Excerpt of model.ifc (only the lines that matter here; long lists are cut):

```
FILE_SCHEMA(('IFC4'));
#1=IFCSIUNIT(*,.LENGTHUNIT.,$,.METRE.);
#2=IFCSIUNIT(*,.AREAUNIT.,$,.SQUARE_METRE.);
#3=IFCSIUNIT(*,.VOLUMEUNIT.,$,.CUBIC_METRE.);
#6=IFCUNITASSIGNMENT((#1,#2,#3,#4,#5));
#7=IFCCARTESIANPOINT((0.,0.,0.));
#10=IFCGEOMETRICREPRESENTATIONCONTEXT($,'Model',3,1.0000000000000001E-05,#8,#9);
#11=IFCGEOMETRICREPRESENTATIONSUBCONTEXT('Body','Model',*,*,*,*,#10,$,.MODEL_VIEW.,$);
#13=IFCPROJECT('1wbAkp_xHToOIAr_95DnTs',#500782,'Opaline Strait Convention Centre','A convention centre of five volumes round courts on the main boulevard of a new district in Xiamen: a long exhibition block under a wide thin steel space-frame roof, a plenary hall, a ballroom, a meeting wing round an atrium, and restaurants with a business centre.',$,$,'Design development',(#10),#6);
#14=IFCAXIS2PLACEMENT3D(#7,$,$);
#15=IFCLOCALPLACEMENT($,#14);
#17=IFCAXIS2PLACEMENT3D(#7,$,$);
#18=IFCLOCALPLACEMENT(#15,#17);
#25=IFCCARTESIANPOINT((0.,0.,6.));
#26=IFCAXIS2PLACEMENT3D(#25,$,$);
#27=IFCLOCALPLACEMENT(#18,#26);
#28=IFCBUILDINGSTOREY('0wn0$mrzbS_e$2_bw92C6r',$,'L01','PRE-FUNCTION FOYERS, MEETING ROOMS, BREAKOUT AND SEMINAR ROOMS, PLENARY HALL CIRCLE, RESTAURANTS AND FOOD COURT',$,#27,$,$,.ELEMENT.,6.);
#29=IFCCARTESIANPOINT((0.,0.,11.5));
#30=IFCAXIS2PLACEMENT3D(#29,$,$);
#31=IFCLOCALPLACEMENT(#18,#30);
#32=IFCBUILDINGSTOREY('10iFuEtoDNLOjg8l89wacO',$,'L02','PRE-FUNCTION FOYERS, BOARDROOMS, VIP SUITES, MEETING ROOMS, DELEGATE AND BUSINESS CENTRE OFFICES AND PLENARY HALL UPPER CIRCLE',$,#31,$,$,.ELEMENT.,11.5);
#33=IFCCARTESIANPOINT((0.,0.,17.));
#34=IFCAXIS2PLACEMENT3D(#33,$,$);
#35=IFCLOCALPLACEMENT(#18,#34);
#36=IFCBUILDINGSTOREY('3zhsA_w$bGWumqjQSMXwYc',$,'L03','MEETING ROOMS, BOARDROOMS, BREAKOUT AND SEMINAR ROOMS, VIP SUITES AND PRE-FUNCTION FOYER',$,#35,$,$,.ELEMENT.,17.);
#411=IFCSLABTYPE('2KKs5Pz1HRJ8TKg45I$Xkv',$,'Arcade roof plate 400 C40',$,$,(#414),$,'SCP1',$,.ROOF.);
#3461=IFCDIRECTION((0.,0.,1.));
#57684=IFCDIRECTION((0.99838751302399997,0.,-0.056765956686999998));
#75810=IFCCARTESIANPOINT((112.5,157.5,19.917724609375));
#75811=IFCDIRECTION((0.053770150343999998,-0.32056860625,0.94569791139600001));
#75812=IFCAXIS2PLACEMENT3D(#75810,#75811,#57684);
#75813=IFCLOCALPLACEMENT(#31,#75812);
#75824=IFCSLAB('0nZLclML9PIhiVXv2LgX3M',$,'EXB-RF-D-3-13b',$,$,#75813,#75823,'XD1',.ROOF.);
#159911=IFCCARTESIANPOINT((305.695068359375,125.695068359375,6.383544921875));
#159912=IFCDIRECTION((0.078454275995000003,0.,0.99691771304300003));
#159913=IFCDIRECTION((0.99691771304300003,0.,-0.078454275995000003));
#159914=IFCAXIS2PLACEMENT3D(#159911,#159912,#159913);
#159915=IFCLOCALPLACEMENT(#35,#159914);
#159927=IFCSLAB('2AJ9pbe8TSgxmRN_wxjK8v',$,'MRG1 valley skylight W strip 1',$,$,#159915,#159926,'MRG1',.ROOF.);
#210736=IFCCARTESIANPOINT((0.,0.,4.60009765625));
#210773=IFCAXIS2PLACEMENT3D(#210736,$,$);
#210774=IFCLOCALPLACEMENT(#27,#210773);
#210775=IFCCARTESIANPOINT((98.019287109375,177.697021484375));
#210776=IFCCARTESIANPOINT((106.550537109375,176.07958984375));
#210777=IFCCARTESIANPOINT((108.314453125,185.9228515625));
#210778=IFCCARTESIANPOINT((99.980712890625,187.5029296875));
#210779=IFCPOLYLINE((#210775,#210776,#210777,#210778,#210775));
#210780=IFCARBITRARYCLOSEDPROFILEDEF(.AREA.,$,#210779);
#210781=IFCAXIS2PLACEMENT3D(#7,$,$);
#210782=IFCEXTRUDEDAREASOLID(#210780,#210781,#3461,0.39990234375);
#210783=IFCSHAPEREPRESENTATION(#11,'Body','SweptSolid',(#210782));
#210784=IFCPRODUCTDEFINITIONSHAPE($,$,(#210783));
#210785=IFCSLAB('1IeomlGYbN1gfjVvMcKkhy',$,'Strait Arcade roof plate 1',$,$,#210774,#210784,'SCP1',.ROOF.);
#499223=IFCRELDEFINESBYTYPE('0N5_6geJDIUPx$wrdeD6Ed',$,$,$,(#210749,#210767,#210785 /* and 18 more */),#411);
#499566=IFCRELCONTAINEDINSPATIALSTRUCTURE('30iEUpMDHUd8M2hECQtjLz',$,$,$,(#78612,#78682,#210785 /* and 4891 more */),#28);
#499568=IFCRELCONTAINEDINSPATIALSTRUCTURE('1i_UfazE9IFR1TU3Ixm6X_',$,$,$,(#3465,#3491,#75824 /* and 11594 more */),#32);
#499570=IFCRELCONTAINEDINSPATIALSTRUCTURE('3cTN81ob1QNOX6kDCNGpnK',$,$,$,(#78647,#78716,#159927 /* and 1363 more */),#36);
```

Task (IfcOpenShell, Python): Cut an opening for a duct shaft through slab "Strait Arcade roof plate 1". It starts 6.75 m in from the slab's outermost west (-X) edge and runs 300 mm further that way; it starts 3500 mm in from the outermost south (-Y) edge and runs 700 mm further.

```python
import numpy as np
import ifcopenshell
import ifcopenshell.api.feature
import ifcopenshell.api.geometry
import ifcopenshell.api.root
import ifcopenshell.geom
import ifcopenshell.util.placement
import ifcopenshell.util.representation
import ifcopenshell.util.shape
import ifcopenshell.util.unit

model = ifcopenshell.open("model.ifc")
unit_scale = ifcopenshell.util.unit.calculate_unit_scale(model)
settings = ifcopenshell.geom.settings()


def volume(element):
    """Net volume in cubic metres, openings subtracted."""
    shape = ifcopenshell.geom.create_shape(settings, element)
    return ifcopenshell.util.shape.get_volume(shape.geometry)


slab = model.by_guid("1IeomlGYbN1gfjVvMcKkhy")
before = volume(slab)

# Extent in the slab's own axes, in metres. The edges named are its -X and -Y sides.
slab_shape = ifcopenshell.geom.create_shape(settings, slab)
vertices = ifcopenshell.util.shape.get_vertices(slab_shape.geometry)
x_min, y_min, bottom = vertices.min(axis=0)
top = vertices[:, 2].max()

opening = ifcopenshell.api.root.create_entity(model, ifc_class="IfcOpeningElement", name="Duct shaft opening", predefined_type="OPENING")
context = ifcopenshell.util.representation.get_context(model, "Model", "Body", "MODEL_VIEW")
width, depth = 0.3, 0.7
outline = [(0.0, 0.0), (width, 0.0), (width, depth), (0.0, depth), (0.0, 0.0)]
# Overshoot both faces by 50 mm so the cut is clean.
shape = ifcopenshell.api.geometry.add_slab_representation(
    model, context=context, depth=top - bottom + 0.1, polyline=outline
)
ifcopenshell.api.geometry.assign_representation(model, product=opening, representation=shape)

matrix = ifcopenshell.util.placement.get_local_placement(slab.ObjectPlacement)
matrix[:, 3] = matrix @ np.append(np.array([x_min + 6.75, y_min + 3.5, bottom - 0.05]) / unit_scale, 1.0)
ifcopenshell.api.geometry.edit_object_placement(model, product=opening, matrix=matrix, is_si=False)
ifcopenshell.api.feature.add_feature(model, feature=opening, element=slab)

after = volume(slab)

print(f"slab volume {before:.3f} -> {after:.3f} m3")

model.write("model_v2.ifc")
```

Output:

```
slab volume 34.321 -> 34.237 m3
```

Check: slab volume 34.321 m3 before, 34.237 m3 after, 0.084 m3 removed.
